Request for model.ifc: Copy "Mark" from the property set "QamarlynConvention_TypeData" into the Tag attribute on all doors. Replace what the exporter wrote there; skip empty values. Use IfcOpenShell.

First a look at what the model holds.

```python
import ifcopenshell
import ifcopenshell.util.element

model = ifcopenshell.open("model.ifc")
print(model.schema)
doors = model.by_type("IfcDoor")
print(len(doors), "doors")
for e in doors[:8]:
    source = ifcopenshell.util.element.get_pset(e, "QamarlynConvention_TypeData", "Mark")
    target = e.Tag
    print(e.id(), repr(source), repr(target), sep=" | ")
```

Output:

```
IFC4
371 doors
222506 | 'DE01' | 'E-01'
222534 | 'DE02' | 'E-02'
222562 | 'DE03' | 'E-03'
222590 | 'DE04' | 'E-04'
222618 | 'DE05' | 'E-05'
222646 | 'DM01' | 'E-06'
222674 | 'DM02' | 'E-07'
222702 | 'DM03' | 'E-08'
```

```python
import ifcopenshell
import ifcopenshell.util.element

model = ifcopenshell.open("model.ifc")

count = 0
for e in model.by_type("IfcDoor"):
    value = ifcopenshell.util.element.get_pset(e, "QamarlynConvention_TypeData", "Mark")
    current = e.Tag
    if not value or not value.strip() or current == value:
        continue
    e.Tag = value
    count += 1

print(count, "doors updated")

model.write("model_edited.ifc")
```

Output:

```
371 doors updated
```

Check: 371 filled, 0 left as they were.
